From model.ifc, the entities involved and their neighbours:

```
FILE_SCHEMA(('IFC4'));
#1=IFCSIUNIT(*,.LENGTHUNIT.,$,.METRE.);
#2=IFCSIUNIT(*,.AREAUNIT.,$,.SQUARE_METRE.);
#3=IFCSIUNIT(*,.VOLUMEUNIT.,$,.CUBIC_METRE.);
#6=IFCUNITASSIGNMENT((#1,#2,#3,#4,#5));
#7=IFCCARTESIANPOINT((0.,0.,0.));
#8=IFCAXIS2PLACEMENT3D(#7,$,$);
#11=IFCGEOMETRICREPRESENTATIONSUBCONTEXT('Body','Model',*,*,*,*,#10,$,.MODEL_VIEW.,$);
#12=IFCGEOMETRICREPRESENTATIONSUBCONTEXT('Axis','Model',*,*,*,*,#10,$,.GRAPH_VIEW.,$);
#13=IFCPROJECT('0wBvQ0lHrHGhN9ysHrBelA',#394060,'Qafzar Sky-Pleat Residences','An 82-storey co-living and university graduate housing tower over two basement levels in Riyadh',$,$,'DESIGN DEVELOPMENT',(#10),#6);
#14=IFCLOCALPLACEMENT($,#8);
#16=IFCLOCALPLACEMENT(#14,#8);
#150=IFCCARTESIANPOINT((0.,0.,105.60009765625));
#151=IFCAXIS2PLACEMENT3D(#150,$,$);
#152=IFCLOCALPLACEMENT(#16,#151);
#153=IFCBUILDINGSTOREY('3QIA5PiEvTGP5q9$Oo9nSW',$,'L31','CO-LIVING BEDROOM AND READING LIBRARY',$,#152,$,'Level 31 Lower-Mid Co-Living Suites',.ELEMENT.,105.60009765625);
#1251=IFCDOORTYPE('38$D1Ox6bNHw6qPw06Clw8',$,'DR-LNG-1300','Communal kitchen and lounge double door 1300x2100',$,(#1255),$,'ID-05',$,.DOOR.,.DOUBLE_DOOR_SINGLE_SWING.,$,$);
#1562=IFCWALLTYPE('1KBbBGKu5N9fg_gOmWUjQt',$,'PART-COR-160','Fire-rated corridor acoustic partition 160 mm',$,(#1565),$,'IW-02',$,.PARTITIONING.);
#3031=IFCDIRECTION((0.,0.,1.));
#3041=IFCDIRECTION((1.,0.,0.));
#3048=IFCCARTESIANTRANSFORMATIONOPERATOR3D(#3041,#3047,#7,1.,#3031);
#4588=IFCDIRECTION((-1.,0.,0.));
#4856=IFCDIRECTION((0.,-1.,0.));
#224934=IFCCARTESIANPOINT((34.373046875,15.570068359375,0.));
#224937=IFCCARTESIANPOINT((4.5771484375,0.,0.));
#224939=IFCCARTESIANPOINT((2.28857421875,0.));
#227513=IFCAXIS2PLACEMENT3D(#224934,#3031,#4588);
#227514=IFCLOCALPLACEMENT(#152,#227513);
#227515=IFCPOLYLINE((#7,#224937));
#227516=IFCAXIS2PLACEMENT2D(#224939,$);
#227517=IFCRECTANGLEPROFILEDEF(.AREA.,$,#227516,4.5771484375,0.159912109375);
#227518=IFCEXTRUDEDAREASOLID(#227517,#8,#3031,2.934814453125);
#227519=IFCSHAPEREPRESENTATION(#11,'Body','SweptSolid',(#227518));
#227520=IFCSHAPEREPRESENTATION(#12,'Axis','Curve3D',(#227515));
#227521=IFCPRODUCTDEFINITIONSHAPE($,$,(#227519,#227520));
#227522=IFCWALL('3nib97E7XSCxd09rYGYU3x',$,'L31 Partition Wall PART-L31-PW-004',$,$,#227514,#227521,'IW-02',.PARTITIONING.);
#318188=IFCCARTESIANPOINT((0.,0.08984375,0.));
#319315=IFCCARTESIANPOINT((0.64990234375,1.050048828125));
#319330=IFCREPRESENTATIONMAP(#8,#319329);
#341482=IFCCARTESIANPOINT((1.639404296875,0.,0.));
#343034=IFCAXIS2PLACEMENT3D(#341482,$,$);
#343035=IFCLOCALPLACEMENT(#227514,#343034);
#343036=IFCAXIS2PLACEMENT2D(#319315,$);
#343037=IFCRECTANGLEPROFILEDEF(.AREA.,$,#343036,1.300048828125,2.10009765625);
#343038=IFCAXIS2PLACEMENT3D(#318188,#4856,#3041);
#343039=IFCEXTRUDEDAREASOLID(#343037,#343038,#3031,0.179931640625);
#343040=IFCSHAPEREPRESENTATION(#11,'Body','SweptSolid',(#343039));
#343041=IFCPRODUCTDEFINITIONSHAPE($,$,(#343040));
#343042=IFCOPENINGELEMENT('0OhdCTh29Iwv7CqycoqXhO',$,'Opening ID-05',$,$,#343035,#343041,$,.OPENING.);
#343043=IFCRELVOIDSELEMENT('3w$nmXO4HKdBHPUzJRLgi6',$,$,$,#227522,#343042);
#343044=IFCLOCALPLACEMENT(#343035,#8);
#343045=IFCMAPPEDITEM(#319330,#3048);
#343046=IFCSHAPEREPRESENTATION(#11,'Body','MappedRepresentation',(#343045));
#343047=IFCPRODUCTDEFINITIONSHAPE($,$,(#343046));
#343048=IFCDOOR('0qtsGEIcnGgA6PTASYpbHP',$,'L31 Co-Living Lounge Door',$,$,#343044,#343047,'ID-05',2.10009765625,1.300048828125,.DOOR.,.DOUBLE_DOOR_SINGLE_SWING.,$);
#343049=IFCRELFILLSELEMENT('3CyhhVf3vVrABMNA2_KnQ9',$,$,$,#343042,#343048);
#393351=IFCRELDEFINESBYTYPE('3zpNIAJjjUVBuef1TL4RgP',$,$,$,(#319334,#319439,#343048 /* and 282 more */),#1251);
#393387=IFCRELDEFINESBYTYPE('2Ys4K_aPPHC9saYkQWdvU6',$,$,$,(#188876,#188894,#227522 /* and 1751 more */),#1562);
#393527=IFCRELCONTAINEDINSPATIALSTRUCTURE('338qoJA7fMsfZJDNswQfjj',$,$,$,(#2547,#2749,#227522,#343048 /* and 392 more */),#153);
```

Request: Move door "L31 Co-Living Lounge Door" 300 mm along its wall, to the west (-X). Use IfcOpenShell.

```python
import ifcopenshell
import ifcopenshell.api.geometry
import ifcopenshell.util.placement

model = ifcopenshell.open("model.ifc")

door = model.by_guid("0qtsGEIcnGgA6PTASYpbHP")
opening = door.FillsVoids[0].RelatingOpeningElement
wall = opening.VoidsElements[0].RelatingBuildingElement

wall_matrix = ifcopenshell.util.placement.get_local_placement(wall.ObjectPlacement)
shift = wall_matrix[:3, 0] * 0.3
before = ifcopenshell.util.placement.get_local_placement(door.ObjectPlacement)[:3, 3].copy()

# The door is placed relative to its opening, so it follows when the opening moves.
matrix = ifcopenshell.util.placement.get_local_placement(opening.ObjectPlacement)
matrix[:3, 3] += shift
ifcopenshell.api.geometry.edit_object_placement(
    model, product=opening, matrix=matrix, is_si=False, should_transform_children=True
)

after = ifcopenshell.util.placement.get_local_placement(door.ObjectPlacement)[:3, 3]
print("door moved by", (after - before).round(3) + 0.0)

model.write("model_v2.ifc")
```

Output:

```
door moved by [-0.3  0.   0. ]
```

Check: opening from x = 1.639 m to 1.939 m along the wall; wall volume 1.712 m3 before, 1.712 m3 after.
